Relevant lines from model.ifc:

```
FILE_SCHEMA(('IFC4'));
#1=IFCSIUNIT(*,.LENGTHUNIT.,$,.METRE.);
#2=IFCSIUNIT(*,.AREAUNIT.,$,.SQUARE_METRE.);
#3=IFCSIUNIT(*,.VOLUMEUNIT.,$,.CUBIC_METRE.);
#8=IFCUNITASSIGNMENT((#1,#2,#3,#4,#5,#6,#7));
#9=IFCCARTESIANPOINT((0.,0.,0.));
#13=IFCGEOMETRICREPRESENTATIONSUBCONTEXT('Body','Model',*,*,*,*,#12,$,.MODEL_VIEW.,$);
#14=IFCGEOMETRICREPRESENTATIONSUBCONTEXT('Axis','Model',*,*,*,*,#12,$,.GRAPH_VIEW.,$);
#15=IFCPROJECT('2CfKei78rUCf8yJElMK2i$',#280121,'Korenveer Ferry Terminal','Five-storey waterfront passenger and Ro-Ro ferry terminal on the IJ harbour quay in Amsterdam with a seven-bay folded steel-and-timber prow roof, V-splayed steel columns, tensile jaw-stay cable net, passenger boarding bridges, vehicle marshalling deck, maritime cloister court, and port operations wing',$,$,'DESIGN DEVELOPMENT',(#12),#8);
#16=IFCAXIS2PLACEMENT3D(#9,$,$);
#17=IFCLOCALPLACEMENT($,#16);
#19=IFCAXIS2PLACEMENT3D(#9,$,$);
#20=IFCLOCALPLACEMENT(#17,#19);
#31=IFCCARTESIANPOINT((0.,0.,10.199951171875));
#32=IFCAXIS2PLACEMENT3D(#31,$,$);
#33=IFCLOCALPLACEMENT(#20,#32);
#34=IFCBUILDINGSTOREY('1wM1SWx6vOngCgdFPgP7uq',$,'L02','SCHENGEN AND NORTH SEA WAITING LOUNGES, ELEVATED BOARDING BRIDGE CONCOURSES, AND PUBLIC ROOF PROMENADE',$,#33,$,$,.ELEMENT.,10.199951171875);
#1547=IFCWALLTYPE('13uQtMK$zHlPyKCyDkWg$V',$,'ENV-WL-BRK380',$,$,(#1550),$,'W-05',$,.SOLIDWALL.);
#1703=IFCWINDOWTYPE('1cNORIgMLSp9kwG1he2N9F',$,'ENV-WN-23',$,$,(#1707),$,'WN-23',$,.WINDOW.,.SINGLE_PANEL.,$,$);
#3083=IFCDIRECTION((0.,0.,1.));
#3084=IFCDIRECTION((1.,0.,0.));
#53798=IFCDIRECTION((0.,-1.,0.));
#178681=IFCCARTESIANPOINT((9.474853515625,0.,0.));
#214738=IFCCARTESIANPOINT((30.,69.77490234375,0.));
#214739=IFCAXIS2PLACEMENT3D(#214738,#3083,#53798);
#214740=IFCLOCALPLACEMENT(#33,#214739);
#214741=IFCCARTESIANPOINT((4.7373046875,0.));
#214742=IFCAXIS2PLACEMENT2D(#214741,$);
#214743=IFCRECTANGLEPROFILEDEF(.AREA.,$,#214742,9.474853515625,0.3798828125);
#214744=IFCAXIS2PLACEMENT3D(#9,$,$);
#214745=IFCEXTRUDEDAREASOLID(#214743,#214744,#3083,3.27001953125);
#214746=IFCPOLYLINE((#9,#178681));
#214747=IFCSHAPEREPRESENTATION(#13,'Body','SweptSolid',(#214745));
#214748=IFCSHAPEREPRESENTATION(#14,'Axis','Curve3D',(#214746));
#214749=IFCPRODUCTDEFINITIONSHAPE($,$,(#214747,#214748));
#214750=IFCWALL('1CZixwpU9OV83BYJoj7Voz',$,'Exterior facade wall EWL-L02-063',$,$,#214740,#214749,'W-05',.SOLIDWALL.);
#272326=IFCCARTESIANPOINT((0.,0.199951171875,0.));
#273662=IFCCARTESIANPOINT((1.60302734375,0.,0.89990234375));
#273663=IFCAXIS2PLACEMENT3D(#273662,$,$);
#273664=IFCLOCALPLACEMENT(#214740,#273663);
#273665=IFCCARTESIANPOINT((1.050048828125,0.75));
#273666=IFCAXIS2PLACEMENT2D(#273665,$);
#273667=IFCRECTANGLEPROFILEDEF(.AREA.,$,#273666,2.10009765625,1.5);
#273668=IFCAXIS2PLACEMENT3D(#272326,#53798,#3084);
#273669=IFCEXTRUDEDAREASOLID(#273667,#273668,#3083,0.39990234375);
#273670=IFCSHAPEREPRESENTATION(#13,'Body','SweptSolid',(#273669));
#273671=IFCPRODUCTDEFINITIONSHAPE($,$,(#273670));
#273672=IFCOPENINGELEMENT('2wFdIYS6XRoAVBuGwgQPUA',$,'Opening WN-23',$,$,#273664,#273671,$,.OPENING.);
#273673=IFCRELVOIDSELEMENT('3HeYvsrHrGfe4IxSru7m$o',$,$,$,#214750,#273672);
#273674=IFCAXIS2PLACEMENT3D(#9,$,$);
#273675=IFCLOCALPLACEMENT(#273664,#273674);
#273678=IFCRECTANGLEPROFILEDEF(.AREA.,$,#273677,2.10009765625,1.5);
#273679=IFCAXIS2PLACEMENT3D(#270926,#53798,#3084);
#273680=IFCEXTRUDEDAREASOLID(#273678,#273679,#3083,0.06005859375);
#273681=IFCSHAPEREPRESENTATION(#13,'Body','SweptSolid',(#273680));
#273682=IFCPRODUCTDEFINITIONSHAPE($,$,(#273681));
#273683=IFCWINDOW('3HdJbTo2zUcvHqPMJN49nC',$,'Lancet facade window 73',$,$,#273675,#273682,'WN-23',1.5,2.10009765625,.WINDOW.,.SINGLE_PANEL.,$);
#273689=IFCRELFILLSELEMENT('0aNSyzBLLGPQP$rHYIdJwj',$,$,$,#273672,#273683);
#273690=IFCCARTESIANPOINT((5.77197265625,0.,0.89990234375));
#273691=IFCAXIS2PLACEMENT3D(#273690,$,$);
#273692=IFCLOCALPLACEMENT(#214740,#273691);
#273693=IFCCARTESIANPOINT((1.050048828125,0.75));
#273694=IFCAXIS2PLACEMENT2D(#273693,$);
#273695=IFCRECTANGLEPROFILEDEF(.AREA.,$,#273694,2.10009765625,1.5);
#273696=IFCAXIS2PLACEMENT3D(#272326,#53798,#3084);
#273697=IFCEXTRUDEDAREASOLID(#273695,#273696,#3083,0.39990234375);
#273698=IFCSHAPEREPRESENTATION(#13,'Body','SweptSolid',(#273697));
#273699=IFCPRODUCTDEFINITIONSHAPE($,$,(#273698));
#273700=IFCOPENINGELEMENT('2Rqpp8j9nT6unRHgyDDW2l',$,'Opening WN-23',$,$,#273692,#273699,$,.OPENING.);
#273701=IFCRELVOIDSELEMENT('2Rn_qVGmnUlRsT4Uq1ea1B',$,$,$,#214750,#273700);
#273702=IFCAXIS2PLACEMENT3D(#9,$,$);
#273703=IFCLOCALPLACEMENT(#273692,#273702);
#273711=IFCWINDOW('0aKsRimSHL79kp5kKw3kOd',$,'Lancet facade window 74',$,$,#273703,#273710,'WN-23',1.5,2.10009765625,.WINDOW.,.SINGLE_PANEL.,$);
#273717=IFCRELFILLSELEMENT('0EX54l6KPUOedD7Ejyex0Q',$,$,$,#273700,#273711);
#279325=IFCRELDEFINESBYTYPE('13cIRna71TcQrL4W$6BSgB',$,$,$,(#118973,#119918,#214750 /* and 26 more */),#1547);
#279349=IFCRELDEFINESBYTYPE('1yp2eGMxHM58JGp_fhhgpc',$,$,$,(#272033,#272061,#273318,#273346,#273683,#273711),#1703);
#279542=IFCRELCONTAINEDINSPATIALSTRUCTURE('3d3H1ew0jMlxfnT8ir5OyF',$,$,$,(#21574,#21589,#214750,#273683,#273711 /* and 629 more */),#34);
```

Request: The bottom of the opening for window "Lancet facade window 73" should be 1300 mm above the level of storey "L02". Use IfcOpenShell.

```python
import numpy as np
import ifcopenshell
import ifcopenshell.api.geometry
import ifcopenshell.geom
import ifcopenshell.util.element
import ifcopenshell.util.placement
import ifcopenshell.util.shape
import ifcopenshell.util.unit

model = ifcopenshell.open("model.ifc")
unit_scale = ifcopenshell.util.unit.calculate_unit_scale(model)

window = model.by_guid("3HdJbTo2zUcvHqPMJN49nC")
opening = window.FillsVoids[0].RelatingOpeningElement
storey = ifcopenshell.util.element.get_container(window, ifc_class="IfcBuildingStorey")
level = ifcopenshell.util.placement.get_local_placement(storey.ObjectPlacement)[2, 3]

# The opening's origin need not be at the sill, so measure its lowest point.
shape = ifcopenshell.geom.create_shape(ifcopenshell.geom.settings(), opening)
bottom = ifcopenshell.util.shape.get_shape_bottom_elevation(shape, shape.geometry) / unit_scale
dz = level + 1.3 / unit_scale - bottom

shift = np.array([0.0, 0.0, dz])
# The window is placed relative to its opening, so it follows when the opening moves.
matrix = ifcopenshell.util.placement.get_local_placement(opening.ObjectPlacement)
matrix[:3, 3] += shift
ifcopenshell.api.geometry.edit_object_placement(
    model, product=opening, matrix=matrix, is_si=False, should_transform_children=True
)

print(f"moved by {dz * unit_scale:+.3f} m")

model.write("model_updated.ifc")
```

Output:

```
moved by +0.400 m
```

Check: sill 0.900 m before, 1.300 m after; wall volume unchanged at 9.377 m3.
